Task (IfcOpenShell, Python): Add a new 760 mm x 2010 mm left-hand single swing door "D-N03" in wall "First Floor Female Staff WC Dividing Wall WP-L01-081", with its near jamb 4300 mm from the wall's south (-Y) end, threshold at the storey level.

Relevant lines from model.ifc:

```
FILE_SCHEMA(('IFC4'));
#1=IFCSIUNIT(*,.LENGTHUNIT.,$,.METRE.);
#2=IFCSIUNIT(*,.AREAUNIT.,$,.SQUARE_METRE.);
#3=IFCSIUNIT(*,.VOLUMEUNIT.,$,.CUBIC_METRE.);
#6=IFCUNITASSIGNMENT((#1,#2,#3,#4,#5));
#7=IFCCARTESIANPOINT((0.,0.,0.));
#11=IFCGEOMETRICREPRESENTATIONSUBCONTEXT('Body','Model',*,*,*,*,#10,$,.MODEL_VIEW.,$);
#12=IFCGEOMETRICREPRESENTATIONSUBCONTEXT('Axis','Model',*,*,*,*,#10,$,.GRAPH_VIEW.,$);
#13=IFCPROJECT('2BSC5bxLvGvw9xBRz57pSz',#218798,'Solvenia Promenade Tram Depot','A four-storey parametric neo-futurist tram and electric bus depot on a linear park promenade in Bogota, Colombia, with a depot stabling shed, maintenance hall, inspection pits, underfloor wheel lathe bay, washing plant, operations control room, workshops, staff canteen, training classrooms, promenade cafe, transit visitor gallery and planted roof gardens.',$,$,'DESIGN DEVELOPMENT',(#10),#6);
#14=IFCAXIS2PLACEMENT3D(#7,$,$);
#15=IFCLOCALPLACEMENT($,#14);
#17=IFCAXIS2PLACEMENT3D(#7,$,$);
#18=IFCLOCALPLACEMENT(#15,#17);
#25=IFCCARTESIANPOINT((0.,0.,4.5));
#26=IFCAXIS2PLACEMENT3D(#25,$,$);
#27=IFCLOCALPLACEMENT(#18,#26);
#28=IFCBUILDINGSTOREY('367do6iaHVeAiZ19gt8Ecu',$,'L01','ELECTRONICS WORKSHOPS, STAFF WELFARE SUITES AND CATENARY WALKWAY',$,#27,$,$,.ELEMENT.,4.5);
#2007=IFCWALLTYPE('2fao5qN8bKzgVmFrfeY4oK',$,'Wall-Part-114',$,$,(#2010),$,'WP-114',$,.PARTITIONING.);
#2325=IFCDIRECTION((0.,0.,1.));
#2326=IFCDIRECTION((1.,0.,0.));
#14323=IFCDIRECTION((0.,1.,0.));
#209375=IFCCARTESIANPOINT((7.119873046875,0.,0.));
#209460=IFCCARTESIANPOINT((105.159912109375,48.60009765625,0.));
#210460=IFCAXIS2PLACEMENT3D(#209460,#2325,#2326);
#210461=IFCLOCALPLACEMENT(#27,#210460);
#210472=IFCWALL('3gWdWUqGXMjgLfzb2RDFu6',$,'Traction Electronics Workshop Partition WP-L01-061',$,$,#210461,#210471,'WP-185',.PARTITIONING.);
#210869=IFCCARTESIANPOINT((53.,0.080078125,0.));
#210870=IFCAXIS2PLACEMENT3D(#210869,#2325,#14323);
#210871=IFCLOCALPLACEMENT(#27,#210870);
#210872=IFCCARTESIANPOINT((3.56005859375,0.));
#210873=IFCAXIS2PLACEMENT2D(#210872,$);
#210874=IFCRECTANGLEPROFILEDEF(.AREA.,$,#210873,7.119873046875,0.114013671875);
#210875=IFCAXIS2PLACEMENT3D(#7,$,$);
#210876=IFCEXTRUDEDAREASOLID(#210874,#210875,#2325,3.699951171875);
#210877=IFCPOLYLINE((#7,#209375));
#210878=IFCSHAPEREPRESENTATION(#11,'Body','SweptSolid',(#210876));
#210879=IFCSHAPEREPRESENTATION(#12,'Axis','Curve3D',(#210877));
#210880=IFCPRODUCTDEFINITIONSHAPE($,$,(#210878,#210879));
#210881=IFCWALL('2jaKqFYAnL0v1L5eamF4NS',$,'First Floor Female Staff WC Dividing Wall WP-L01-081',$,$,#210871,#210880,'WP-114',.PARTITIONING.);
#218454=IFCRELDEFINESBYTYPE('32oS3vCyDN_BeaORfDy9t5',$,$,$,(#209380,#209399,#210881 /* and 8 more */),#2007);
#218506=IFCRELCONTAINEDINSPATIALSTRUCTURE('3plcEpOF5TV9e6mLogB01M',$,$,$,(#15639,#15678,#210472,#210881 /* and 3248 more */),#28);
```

```python
import numpy as np
import ifcopenshell
import ifcopenshell.api.feature
import ifcopenshell.api.geometry
import ifcopenshell.api.root
import ifcopenshell.api.spatial
import ifcopenshell.geom
import ifcopenshell.util.element
import ifcopenshell.util.placement
import ifcopenshell.util.representation
import ifcopenshell.util.shape
import ifcopenshell.util.unit

model = ifcopenshell.open("model.ifc")
unit_scale = ifcopenshell.util.unit.calculate_unit_scale(model)
settings = ifcopenshell.geom.settings()


def volume(element):
    """Net volume in cubic metres, openings subtracted."""
    shape = ifcopenshell.geom.create_shape(settings, element)
    return ifcopenshell.util.shape.get_volume(shape.geometry)


wall = model.by_id(210881)
storey = ifcopenshell.util.element.get_container(wall, ifc_class="IfcBuildingStorey")
context = ifcopenshell.util.representation.get_context(model, "Model", "Body", "MODEL_VIEW")
before = volume(wall)

width, height, from_end, sill = 0.76, 2.01, 4.3, 0.0  # metres

# The wall runs along its own X axis, and the end named is its -X end.
wall_shape = ifcopenshell.geom.create_shape(settings, wall)
x, y, z = ifcopenshell.util.shape.get_vertices(wall_shape.geometry).T
start = x.min() + from_end
face, thickness = float(y.min()), float(y.max() - y.min())
wall_matrix = ifcopenshell.util.placement.get_local_placement(wall.ObjectPlacement)
level = ifcopenshell.util.placement.get_local_placement(storey.ObjectPlacement)[2, 3]


def in_wall(x, y):
    """Placement at x, y metres in the wall's axes, at sill height."""
    matrix = wall_matrix.copy()
    matrix[:, 3] = wall_matrix @ np.array([x / unit_scale, y / unit_scale, 0.0, 1.0])
    matrix[2, 3] = level + sill / unit_scale
    return matrix


# Opening: a box that overshoots both wall faces by 50 mm.
opening = ifcopenshell.api.root.create_entity(model, ifc_class="IfcOpeningElement", predefined_type="OPENING")
box = ifcopenshell.api.geometry.add_wall_representation(
    model, context=context, length=width, height=height, thickness=thickness + 0.1
)
ifcopenshell.api.geometry.assign_representation(model, product=opening, representation=box)
ifcopenshell.api.geometry.edit_object_placement(model, product=opening, matrix=in_wall(start, face - 0.05), is_si=False)
ifcopenshell.api.feature.add_feature(model, feature=opening, element=wall)

door = ifcopenshell.api.root.create_entity(model, ifc_class="IfcDoor", name="D-N03", predefined_type="DOOR")
door.OverallWidth, door.OverallHeight = width / unit_scale, height / unit_scale
door.OperationType = "SINGLE_SWING_LEFT"
body = ifcopenshell.api.geometry.add_door_representation(
    model,
    context=context,
    overall_width=door.OverallWidth,
    overall_height=door.OverallHeight,
    operation_type="SINGLE_SWING_LEFT",
    lining_properties={"LiningDepth": thickness / unit_scale, "ThresholdDepth": thickness / unit_scale},
)
ifcopenshell.api.geometry.assign_representation(model, product=door, representation=body)
ifcopenshell.api.spatial.assign_container(model, products=[door], relating_structure=storey)
ifcopenshell.api.feature.add_filling(model, opening=opening, element=door)

# The lining spans the wall, so the door starts at the wall face.
ifcopenshell.api.geometry.edit_object_placement(model, product=door, matrix=in_wall(start, face), is_si=False)

after = volume(wall)

print(f"wall volume {before:.3f} -> {after:.3f} m3")

model.write("model_v2.ifc")
```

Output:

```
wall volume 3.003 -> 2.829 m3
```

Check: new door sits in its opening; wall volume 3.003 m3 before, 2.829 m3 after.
